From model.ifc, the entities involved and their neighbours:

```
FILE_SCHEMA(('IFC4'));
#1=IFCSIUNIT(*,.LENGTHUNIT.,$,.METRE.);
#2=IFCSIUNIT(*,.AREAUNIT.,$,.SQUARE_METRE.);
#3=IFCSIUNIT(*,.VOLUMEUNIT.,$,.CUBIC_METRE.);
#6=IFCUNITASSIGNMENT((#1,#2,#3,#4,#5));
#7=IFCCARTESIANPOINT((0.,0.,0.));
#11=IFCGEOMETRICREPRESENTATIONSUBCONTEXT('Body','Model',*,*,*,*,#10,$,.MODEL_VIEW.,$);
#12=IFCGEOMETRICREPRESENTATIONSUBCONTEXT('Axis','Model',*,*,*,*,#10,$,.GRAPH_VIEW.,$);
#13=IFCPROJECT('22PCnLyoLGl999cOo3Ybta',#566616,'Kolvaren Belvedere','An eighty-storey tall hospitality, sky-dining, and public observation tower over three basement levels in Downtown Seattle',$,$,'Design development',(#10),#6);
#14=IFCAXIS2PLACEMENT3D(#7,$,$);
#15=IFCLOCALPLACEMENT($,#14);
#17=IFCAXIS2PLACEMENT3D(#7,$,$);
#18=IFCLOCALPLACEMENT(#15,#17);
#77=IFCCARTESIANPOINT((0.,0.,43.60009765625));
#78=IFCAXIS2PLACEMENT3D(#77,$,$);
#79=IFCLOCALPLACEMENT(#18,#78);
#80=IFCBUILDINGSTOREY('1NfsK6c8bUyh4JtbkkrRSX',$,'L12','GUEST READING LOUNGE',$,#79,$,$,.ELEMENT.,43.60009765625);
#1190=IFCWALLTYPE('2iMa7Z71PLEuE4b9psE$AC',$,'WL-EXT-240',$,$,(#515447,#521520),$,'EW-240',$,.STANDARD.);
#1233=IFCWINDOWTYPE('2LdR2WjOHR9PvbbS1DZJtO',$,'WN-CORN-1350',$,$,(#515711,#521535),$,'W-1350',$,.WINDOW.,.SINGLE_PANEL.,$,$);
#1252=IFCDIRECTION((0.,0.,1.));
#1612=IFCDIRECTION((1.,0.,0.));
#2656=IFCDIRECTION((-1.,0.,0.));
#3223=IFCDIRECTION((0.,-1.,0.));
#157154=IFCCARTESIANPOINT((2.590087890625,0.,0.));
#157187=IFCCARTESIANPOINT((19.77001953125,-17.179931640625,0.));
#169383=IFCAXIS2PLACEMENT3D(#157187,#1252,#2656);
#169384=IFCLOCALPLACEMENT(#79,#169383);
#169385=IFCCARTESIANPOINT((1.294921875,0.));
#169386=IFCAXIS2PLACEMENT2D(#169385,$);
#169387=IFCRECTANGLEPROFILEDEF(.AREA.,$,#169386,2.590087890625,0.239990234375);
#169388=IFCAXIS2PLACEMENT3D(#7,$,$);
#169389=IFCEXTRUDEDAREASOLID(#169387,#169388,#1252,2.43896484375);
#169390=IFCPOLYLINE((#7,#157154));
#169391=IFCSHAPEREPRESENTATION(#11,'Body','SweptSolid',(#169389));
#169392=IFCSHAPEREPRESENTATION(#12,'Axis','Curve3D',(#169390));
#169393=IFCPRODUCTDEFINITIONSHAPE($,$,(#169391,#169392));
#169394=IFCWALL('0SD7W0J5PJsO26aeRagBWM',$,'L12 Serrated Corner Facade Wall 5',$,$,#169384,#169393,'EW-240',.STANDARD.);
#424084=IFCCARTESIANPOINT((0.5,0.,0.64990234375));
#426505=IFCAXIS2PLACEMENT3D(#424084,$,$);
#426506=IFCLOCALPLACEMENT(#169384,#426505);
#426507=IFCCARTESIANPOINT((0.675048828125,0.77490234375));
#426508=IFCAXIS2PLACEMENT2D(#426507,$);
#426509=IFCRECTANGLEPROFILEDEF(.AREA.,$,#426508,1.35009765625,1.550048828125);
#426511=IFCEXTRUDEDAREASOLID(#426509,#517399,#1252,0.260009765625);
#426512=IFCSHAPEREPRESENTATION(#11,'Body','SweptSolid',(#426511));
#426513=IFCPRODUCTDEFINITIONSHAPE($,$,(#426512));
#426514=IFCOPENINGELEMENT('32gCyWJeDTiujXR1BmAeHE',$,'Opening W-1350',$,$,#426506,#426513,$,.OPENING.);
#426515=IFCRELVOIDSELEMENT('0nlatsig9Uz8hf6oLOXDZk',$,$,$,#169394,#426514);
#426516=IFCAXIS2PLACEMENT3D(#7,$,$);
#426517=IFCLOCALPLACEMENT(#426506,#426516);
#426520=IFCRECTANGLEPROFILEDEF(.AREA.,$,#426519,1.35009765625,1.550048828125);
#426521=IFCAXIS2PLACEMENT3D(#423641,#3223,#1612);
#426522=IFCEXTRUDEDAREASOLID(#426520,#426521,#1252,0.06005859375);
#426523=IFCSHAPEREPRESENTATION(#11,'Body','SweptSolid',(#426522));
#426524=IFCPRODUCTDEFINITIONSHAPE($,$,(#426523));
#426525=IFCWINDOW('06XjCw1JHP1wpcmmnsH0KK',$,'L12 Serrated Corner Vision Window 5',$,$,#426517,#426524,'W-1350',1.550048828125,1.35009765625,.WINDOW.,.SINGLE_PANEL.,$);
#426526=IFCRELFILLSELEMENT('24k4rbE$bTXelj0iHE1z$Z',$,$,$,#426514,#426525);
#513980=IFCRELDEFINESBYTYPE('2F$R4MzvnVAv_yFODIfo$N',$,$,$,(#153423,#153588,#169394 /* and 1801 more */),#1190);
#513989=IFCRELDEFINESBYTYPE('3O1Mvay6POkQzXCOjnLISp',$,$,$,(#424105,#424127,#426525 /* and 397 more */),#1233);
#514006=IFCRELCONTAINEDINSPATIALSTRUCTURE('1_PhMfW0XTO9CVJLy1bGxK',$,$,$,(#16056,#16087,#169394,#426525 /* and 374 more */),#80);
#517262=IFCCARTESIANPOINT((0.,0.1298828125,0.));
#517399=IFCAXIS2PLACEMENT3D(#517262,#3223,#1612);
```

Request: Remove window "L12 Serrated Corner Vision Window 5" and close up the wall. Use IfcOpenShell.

```python
import ifcopenshell
import ifcopenshell.api.feature
import ifcopenshell.api.root
import ifcopenshell.geom
import ifcopenshell.util.shape

model = ifcopenshell.open("model.ifc")
settings = ifcopenshell.geom.settings()


def volume(element):
    """Net volume in cubic metres, openings subtracted."""
    shape = ifcopenshell.geom.create_shape(settings, element)
    return ifcopenshell.util.shape.get_volume(shape.geometry)


window = model.by_id(426525)
opening = window.FillsVoids[0].RelatingOpeningElement
wall = opening.VoidsElements[0].RelatingBuildingElement
before = volume(wall)

ifcopenshell.api.root.remove_product(model, product=window)
ifcopenshell.api.feature.remove_feature(model, feature=opening)

after = volume(wall)

print(f"wall volume {before:.3f} -> {after:.3f} m3")

model.write("model_edited.ifc")
```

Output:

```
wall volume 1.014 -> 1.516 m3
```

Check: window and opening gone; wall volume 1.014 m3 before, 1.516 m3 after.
